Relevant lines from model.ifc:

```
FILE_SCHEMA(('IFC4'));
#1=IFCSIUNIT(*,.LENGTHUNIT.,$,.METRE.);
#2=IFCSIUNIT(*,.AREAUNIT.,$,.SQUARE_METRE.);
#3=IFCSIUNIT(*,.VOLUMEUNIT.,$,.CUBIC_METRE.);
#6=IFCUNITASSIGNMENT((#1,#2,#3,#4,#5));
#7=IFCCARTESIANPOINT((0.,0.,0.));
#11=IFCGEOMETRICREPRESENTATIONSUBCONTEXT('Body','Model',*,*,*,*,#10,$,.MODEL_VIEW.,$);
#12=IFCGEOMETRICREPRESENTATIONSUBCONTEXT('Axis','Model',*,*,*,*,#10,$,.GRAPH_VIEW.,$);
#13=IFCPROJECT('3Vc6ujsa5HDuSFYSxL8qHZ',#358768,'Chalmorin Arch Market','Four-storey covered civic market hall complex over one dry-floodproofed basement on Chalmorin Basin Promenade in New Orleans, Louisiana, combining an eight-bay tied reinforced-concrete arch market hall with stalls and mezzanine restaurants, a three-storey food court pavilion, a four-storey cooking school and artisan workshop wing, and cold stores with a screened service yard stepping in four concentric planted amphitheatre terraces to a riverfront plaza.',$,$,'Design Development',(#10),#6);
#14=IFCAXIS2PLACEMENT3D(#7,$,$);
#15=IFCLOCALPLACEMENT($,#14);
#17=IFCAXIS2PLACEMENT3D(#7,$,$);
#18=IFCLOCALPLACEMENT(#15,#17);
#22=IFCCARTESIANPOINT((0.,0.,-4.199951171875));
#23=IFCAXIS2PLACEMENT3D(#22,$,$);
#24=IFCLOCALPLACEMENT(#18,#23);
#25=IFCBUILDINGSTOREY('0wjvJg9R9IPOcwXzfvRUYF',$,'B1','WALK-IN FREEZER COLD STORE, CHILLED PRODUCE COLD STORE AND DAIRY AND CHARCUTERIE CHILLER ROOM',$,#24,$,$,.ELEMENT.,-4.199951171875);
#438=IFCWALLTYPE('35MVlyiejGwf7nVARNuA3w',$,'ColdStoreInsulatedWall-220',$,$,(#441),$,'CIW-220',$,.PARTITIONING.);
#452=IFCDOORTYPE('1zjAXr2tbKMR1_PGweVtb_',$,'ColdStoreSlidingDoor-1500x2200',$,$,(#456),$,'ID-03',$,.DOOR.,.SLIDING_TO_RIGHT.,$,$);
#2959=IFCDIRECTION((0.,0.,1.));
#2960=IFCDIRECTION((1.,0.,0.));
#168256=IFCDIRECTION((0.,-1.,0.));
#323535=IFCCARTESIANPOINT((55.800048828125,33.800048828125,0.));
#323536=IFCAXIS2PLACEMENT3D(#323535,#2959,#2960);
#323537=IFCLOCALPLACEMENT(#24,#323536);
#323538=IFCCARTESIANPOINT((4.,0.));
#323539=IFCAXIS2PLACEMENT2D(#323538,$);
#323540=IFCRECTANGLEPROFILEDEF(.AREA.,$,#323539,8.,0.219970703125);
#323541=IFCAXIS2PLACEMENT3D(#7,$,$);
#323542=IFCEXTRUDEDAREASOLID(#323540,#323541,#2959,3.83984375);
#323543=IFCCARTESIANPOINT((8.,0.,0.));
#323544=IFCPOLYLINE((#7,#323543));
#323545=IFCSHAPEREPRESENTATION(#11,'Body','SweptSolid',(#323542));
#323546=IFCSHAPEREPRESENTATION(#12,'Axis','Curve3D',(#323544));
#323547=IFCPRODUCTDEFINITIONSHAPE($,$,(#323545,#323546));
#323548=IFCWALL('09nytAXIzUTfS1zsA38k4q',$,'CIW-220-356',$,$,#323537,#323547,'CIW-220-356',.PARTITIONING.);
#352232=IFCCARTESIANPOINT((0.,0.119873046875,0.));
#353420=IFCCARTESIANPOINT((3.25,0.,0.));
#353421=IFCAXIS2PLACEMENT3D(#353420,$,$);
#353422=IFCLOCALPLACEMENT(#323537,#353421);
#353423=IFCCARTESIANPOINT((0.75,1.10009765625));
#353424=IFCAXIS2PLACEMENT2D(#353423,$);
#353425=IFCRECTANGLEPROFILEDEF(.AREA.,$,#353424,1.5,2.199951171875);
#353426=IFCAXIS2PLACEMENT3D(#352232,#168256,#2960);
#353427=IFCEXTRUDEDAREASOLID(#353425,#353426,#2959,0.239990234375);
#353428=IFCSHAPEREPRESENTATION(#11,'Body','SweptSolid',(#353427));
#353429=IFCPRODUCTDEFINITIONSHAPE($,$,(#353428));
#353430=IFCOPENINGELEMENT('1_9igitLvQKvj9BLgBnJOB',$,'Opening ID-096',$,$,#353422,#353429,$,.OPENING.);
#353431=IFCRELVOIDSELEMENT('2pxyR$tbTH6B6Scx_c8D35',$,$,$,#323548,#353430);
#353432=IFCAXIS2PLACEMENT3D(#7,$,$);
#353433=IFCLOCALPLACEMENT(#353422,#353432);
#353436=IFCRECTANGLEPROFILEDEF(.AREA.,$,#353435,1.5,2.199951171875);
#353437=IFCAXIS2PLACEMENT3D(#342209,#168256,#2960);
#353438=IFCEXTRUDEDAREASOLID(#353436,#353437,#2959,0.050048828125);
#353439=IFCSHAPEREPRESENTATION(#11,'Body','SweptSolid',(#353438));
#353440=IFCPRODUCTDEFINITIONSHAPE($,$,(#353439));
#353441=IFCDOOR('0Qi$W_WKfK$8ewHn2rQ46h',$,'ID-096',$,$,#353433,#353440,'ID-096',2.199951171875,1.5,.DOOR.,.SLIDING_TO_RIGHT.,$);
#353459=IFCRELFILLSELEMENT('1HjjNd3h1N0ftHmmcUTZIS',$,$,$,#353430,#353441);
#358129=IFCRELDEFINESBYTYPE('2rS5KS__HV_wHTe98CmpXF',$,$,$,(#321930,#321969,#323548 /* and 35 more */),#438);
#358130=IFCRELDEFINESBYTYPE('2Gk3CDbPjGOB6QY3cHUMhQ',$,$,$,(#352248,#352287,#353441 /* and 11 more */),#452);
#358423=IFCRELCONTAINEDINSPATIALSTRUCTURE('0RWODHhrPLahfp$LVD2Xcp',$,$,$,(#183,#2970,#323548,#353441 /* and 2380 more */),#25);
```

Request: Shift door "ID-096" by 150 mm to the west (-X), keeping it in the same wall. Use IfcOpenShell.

```python
import ifcopenshell
import ifcopenshell.api.geometry
import ifcopenshell.util.placement

model = ifcopenshell.open("model.ifc")

door = model.by_guid("0Qi$W_WKfK$8ewHn2rQ46h")
opening = door.FillsVoids[0].RelatingOpeningElement
wall = opening.VoidsElements[0].RelatingBuildingElement

wall_matrix = ifcopenshell.util.placement.get_local_placement(wall.ObjectPlacement)
shift = wall_matrix[:3, 0] * -0.15
before = ifcopenshell.util.placement.get_local_placement(door.ObjectPlacement)[:3, 3].copy()

# The door is placed relative to its opening, so it follows when the opening moves.
matrix = ifcopenshell.util.placement.get_local_placement(opening.ObjectPlacement)
matrix[:3, 3] += shift
ifcopenshell.api.geometry.edit_object_placement(
    model, product=opening, matrix=matrix, is_si=False, should_transform_children=True
)

after = ifcopenshell.util.placement.get_local_placement(door.ObjectPlacement)[:3, 3]
print("door moved by", (after - before).round(3) + 0.0)

model.write("model-out.ifc")
```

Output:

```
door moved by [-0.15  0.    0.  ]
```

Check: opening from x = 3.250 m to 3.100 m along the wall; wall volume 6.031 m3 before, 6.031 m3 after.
